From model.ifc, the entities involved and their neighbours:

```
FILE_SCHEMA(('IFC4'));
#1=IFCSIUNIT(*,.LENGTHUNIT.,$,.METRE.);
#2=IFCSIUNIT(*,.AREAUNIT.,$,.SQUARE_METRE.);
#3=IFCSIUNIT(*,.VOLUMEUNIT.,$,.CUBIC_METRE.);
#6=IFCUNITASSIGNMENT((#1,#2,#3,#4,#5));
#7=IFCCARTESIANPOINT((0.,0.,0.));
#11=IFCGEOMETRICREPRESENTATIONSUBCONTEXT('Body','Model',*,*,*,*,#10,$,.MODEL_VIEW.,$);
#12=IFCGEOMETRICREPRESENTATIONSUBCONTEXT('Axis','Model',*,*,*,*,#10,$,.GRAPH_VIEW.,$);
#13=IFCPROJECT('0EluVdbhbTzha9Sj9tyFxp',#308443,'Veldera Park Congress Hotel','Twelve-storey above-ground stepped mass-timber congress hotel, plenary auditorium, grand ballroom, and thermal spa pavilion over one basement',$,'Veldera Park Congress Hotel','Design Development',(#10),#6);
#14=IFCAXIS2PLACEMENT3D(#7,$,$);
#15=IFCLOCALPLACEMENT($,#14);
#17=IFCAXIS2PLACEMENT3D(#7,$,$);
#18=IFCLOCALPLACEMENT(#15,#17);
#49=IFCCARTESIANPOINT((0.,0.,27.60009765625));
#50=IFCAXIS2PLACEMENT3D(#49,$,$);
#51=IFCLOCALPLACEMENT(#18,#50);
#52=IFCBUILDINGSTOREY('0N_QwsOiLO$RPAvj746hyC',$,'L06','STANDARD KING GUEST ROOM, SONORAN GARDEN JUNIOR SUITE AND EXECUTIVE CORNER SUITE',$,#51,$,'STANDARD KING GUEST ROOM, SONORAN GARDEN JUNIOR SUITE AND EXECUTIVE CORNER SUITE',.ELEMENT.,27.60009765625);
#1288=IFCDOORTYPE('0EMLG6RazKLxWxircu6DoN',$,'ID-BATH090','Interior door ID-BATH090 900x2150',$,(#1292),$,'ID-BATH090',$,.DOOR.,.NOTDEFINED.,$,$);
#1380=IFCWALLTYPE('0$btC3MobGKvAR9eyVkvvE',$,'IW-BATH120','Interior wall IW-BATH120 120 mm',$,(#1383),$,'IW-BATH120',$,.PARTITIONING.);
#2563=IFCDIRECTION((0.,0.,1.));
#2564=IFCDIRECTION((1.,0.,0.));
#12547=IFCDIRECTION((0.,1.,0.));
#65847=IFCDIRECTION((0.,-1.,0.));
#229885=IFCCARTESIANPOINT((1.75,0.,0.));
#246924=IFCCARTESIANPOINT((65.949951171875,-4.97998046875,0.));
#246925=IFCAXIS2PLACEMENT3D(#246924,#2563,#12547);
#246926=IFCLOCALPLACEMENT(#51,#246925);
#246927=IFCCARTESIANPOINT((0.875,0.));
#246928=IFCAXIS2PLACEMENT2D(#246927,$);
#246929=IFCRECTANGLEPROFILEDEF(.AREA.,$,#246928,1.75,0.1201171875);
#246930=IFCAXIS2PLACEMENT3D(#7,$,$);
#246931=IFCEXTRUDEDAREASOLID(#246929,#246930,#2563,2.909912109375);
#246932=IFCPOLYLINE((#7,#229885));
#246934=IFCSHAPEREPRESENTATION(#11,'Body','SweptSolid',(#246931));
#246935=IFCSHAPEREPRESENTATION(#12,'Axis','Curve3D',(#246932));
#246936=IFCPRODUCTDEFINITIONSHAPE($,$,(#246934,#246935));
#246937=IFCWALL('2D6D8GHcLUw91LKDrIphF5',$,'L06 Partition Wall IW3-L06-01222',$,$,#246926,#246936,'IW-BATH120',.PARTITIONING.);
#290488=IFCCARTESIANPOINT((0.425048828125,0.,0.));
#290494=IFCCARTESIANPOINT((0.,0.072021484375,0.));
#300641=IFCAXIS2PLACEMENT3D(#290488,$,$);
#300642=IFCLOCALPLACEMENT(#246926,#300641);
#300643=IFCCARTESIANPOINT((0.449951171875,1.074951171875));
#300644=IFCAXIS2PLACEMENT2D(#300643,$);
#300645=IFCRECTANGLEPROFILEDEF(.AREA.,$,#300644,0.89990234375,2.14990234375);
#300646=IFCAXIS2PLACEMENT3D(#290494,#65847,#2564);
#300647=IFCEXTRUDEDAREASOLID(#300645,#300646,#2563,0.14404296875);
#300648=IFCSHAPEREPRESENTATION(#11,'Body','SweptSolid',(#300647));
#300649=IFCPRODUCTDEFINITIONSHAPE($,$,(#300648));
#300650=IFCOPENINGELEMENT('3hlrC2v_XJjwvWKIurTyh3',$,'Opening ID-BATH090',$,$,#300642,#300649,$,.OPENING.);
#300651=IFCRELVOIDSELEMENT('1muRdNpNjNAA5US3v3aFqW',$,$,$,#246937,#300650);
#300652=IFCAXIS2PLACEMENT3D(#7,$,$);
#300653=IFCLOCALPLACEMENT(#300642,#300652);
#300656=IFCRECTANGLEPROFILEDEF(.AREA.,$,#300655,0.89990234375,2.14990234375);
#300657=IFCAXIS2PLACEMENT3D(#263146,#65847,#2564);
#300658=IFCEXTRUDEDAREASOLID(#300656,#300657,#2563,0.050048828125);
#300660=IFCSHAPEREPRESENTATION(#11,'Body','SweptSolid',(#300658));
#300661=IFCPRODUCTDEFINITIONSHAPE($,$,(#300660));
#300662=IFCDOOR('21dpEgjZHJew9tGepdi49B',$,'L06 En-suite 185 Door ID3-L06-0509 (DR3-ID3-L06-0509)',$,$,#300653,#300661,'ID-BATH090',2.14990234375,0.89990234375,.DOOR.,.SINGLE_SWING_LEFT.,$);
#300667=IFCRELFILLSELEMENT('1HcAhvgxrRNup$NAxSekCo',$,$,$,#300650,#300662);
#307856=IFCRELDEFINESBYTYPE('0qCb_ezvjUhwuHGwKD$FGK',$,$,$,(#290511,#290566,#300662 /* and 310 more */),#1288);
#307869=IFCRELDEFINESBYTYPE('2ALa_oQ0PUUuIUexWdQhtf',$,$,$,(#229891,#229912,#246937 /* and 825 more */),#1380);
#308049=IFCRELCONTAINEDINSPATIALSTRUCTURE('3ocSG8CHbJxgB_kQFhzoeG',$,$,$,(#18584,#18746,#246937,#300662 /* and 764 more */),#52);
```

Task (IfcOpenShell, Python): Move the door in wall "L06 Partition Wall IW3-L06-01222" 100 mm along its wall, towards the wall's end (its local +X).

```python
import ifcopenshell
import ifcopenshell.api.geometry
import ifcopenshell.util.placement
import ifcopenshell.util.unit

model = ifcopenshell.open("model.ifc")
unit_scale = ifcopenshell.util.unit.calculate_unit_scale(model)

door = model.by_guid("21dpEgjZHJew9tGepdi49B")
opening = door.FillsVoids[0].RelatingOpeningElement
wall = opening.VoidsElements[0].RelatingBuildingElement

wall_matrix = ifcopenshell.util.placement.get_local_placement(wall.ObjectPlacement)
shift = wall_matrix[:3, 0] * 0.1 / unit_scale
before = ifcopenshell.util.placement.get_local_placement(door.ObjectPlacement)[:3, 3].copy()

# The door is placed relative to its opening, so it follows when the opening moves.
matrix = ifcopenshell.util.placement.get_local_placement(opening.ObjectPlacement)
matrix[:3, 3] += shift
ifcopenshell.api.geometry.edit_object_placement(
    model, product=opening, matrix=matrix, is_si=False, should_transform_children=True
)

after = ifcopenshell.util.placement.get_local_placement(door.ObjectPlacement)[:3, 3]
print("door moved by", (after - before).round(3) + 0.0)

model.write("model_edited.ifc")
```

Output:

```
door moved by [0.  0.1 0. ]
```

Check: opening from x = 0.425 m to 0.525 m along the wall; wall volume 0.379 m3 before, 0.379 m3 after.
